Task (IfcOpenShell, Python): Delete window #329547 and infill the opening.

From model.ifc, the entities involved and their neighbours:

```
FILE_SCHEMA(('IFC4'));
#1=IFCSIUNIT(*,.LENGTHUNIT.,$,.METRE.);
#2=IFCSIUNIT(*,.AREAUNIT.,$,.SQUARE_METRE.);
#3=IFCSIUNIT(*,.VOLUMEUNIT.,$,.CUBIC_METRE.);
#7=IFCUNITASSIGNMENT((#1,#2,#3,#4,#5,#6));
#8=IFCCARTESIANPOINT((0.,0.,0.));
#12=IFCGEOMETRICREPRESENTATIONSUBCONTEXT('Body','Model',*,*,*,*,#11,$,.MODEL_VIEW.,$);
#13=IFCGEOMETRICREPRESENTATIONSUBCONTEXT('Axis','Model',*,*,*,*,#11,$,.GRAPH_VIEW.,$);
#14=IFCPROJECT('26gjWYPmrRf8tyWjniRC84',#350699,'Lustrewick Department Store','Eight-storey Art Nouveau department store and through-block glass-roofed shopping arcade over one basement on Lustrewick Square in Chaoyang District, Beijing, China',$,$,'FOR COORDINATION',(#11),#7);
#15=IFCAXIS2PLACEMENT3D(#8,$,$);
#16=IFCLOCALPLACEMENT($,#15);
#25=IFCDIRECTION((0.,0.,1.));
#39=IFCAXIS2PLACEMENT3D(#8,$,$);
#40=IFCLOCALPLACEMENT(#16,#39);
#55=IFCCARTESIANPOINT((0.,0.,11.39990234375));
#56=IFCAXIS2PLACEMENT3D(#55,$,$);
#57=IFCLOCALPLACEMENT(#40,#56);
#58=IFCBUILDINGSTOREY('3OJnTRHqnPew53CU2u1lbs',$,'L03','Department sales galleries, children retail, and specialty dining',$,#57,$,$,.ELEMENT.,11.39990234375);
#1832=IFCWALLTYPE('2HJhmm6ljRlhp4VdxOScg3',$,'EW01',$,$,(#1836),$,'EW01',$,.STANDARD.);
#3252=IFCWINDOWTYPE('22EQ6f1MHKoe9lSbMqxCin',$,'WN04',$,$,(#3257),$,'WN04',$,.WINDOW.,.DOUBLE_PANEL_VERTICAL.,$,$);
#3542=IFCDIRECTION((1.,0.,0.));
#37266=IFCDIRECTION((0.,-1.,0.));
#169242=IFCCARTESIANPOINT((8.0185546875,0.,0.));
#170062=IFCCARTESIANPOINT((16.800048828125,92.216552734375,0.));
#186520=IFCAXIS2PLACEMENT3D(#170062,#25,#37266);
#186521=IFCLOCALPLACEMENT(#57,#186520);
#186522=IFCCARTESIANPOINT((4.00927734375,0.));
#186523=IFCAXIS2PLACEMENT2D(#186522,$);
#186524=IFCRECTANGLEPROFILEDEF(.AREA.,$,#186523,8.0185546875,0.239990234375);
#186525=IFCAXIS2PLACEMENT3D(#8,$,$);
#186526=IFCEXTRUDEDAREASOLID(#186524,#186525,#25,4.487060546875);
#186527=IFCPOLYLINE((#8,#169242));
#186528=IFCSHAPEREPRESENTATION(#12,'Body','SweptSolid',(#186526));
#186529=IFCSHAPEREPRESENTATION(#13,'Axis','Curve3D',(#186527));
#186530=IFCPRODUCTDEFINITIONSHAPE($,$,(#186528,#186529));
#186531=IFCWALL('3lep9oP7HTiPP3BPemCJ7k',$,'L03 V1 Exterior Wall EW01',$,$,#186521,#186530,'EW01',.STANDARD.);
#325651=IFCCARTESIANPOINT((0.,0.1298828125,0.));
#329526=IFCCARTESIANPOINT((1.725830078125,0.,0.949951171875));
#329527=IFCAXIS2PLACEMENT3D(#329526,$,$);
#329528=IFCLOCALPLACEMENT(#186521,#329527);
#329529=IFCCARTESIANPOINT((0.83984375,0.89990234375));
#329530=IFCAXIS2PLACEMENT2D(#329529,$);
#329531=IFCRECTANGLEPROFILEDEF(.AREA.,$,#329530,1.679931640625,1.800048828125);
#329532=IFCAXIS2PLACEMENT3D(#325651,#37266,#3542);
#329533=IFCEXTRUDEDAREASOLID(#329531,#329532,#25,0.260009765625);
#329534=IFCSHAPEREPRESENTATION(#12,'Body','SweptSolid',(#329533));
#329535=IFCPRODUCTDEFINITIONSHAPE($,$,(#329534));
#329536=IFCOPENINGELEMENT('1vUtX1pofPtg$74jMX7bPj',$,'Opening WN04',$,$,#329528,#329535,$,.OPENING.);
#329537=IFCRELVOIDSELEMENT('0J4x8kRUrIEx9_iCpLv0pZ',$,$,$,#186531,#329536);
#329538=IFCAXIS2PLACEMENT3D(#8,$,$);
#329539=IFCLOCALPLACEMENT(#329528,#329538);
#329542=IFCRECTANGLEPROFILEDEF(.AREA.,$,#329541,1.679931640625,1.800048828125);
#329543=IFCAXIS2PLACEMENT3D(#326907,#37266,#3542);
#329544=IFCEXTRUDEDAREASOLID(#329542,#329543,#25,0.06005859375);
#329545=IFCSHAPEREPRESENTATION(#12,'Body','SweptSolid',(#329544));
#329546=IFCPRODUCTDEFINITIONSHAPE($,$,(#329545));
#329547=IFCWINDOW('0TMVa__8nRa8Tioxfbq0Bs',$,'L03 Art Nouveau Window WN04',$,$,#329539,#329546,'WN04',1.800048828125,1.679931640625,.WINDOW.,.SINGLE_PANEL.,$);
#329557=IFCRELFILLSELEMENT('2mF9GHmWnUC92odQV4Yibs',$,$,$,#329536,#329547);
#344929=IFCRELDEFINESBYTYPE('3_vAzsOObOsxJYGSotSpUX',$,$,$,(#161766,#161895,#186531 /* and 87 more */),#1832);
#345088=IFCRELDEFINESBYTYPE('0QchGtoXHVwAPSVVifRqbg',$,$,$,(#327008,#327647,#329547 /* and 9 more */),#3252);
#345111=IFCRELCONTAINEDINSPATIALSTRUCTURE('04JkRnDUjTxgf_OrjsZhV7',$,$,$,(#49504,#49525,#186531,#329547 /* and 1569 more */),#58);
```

```python
import ifcopenshell
import ifcopenshell.api.feature
import ifcopenshell.api.root
import ifcopenshell.geom
import ifcopenshell.util.shape

model = ifcopenshell.open("model.ifc")
settings = ifcopenshell.geom.settings()


def volume(element):
    """Net volume in cubic metres, openings subtracted."""
    shape = ifcopenshell.geom.create_shape(settings, element)
    return ifcopenshell.util.shape.get_volume(shape.geometry)


window = model.by_id(329547)
opening = window.FillsVoids[0].RelatingOpeningElement
wall = opening.VoidsElements[0].RelatingBuildingElement
before = volume(wall)

ifcopenshell.api.root.remove_product(model, product=window)
ifcopenshell.api.feature.remove_feature(model, feature=opening)

after = volume(wall)

print(f"wall volume {before:.3f} -> {after:.3f} m3")

model.write("model_updated.ifc")
```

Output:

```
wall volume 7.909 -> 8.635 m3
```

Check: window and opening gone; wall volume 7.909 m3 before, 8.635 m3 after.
